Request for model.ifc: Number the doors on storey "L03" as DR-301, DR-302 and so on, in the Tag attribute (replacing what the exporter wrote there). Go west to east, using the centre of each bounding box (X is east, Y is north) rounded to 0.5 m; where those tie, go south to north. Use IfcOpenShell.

First a look at what the model holds.

```python
import ifcopenshell
import ifcopenshell.util.element
import ifcopenshell.util.placement

model = ifcopenshell.open("model.ifc")
print(model.schema)
storey = next(s for s in model.by_type("IfcBuildingStorey") if s.Name == "L03")
doors = [e for e in ifcopenshell.util.element.get_decomposition(storey) if e.is_a("IfcDoor")]
for e in sorted(doors, key=lambda e: e.id()):
    origin = ifcopenshell.util.placement.get_local_placement(e.ObjectPlacement)[:3, 3]
    print(e.id(), e.Tag, e.Name, origin.round(2) + 0.0, sep=" | ")
```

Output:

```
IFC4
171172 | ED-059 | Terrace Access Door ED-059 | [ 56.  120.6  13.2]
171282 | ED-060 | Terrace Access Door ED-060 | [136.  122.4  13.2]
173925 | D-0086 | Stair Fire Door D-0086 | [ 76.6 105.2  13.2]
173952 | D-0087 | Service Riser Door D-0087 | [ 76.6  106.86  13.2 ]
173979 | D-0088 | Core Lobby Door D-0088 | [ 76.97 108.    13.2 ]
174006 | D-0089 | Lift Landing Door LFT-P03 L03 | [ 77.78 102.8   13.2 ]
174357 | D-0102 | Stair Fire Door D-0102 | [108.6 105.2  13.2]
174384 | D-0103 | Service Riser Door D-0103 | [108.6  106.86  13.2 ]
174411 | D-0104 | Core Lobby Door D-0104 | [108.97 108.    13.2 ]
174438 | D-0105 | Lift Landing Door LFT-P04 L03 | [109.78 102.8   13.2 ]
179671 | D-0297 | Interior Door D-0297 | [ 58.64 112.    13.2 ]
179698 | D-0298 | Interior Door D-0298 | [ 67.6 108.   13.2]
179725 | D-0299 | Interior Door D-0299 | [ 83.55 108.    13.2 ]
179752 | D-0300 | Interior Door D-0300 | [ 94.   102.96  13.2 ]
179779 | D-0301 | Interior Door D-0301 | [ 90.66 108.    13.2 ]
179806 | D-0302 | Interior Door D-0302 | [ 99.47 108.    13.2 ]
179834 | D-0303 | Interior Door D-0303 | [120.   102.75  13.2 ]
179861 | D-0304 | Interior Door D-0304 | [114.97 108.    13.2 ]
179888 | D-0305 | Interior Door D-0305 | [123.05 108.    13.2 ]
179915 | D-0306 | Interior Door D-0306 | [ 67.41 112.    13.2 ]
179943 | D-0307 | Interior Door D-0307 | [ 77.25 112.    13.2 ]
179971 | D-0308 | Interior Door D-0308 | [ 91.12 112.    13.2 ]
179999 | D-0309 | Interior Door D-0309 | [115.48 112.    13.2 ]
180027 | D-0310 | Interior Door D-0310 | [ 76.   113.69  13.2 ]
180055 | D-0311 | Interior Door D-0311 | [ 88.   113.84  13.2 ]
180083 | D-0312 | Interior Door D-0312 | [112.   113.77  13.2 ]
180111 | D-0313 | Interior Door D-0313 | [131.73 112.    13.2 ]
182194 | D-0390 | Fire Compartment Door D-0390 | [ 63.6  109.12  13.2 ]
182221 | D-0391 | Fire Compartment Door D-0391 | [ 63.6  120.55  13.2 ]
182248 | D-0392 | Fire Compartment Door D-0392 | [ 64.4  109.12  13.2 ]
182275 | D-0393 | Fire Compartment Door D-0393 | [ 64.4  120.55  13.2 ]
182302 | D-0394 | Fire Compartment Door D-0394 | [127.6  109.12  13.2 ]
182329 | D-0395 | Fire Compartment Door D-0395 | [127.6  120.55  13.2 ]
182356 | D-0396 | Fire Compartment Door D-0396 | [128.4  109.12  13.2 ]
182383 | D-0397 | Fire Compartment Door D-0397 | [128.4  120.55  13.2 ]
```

```python
import ifcopenshell
import ifcopenshell.geom
import ifcopenshell.util.element
import ifcopenshell.util.shape

model = ifcopenshell.open("model.ifc")
settings = ifcopenshell.geom.settings()
settings.set("use-world-coords", True)


def centre(element):
    shape = ifcopenshell.geom.create_shape(settings, element)
    return ifcopenshell.util.shape.get_bbox_centroid(shape.geometry)


storey = next(s for s in model.by_type("IfcBuildingStorey") if s.Name == "L03")
doors = [e for e in ifcopenshell.util.element.get_decomposition(storey) if e.is_a("IfcDoor")]

# Insertion points can sit at a corner or the storey origin, so sort by the geometry (in metres).
centres = {e: centre(e) for e in doors}
doors.sort(key=lambda e: (round(centres[e][0] / 0.5), centres[e][1]))

for i, e in enumerate(doors, start=1):
    number = f"DR-3{i:02d}"
    e.Tag = number
    print(e.id(), number)

model.write("model_rev.ifc")
```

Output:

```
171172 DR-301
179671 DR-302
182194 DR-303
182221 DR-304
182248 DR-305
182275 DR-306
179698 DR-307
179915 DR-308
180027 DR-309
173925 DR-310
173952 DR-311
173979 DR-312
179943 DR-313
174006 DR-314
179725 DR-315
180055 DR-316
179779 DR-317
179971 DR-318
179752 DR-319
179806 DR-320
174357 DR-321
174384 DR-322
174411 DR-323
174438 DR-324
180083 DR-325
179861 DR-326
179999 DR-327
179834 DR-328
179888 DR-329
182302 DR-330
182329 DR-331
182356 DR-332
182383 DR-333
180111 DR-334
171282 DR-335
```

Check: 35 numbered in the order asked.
